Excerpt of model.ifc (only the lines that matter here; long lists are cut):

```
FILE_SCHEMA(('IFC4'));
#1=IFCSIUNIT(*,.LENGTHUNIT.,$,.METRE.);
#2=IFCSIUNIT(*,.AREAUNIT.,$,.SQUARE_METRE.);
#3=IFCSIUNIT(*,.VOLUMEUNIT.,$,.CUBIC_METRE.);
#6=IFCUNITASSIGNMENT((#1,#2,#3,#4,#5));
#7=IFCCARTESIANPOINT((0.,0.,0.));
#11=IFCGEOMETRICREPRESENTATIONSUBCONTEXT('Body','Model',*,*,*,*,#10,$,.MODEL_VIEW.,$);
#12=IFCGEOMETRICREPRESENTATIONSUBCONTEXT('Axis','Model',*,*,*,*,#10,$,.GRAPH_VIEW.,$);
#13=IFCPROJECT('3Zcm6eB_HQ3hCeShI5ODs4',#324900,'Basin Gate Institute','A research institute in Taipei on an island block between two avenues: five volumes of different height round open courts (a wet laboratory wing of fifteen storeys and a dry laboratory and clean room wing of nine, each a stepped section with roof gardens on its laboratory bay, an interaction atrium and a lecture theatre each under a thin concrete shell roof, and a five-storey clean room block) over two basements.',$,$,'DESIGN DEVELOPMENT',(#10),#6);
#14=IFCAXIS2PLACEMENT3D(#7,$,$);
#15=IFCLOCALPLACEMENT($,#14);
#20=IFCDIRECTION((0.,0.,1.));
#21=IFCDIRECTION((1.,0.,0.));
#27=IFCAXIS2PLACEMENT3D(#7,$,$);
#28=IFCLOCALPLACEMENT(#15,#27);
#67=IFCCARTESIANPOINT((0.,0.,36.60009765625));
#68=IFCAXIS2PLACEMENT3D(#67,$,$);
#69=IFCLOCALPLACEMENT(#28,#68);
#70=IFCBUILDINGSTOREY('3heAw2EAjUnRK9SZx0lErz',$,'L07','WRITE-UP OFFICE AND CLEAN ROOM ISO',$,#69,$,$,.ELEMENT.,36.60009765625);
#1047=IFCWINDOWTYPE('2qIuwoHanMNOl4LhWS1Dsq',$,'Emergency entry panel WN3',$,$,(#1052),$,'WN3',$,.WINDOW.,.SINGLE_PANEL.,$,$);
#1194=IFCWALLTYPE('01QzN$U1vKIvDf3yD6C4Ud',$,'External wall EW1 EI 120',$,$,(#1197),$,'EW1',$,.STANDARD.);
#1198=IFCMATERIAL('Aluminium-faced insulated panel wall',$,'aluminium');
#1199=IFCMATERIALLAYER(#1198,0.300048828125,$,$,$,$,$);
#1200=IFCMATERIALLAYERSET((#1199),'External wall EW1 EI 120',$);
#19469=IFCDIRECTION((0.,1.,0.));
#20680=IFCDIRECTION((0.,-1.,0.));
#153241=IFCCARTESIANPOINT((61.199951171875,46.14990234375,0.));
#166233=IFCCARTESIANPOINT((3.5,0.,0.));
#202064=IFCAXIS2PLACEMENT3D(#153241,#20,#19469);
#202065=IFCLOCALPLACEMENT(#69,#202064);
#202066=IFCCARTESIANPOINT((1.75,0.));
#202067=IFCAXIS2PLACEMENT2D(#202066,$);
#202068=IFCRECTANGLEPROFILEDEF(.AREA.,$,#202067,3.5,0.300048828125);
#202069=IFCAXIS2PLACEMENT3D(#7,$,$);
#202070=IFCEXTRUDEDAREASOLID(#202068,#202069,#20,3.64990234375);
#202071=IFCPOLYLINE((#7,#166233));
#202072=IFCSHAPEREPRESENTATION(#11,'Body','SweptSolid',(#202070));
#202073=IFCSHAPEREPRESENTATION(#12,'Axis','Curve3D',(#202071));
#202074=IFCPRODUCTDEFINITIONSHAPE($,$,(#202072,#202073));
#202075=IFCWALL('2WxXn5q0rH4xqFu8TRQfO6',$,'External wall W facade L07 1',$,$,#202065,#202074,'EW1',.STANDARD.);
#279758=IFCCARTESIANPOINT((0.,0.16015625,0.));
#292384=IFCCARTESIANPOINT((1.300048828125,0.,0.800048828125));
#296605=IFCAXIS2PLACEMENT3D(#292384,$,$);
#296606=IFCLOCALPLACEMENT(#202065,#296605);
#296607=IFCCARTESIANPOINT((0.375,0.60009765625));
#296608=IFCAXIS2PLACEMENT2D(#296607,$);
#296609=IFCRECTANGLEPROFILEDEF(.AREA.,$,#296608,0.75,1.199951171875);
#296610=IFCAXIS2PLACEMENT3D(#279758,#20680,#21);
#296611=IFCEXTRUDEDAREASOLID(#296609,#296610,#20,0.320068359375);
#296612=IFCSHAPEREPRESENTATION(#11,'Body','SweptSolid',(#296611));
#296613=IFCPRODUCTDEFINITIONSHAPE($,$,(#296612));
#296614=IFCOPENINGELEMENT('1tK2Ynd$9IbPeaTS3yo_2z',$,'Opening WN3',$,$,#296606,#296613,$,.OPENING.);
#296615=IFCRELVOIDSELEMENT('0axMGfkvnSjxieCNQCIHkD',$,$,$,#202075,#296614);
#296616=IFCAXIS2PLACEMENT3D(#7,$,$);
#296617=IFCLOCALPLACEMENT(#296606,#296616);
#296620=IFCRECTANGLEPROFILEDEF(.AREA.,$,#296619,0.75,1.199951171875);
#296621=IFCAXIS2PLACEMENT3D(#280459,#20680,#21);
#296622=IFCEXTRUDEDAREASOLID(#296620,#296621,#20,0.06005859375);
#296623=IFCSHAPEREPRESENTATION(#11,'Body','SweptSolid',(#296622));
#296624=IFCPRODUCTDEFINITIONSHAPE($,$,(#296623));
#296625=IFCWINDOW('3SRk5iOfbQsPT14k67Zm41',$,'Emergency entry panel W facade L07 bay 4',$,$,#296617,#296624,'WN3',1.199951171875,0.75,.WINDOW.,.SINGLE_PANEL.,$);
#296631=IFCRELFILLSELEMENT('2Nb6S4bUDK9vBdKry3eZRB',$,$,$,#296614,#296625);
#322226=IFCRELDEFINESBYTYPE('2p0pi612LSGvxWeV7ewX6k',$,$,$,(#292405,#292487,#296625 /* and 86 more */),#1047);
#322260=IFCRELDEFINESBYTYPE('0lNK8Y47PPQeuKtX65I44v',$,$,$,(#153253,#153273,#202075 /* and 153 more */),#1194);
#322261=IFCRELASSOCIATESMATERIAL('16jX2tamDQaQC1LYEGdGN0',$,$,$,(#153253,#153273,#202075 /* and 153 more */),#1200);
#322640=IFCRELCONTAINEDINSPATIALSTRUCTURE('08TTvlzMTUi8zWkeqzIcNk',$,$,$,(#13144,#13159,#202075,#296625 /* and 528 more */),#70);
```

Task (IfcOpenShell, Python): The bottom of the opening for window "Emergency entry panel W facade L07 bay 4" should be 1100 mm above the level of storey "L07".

```python
import numpy as np
import ifcopenshell
import ifcopenshell.api.geometry
import ifcopenshell.geom
import ifcopenshell.util.element
import ifcopenshell.util.placement
import ifcopenshell.util.shape
import ifcopenshell.util.unit

model = ifcopenshell.open("model.ifc")
unit_scale = ifcopenshell.util.unit.calculate_unit_scale(model)

window = model.by_guid("3SRk5iOfbQsPT14k67Zm41")
opening = window.FillsVoids[0].RelatingOpeningElement
storey = ifcopenshell.util.element.get_container(window, ifc_class="IfcBuildingStorey")
level = ifcopenshell.util.placement.get_local_placement(storey.ObjectPlacement)[2, 3]

# The opening's origin need not be at the sill, so measure its lowest point.
shape = ifcopenshell.geom.create_shape(ifcopenshell.geom.settings(), opening)
bottom = ifcopenshell.util.shape.get_shape_bottom_elevation(shape, shape.geometry) / unit_scale
dz = level + 1.1 / unit_scale - bottom

shift = np.array([0.0, 0.0, dz])
# The window is placed relative to its opening, so it follows when the opening moves.
matrix = ifcopenshell.util.placement.get_local_placement(opening.ObjectPlacement)
matrix[:3, 3] += shift
ifcopenshell.api.geometry.edit_object_placement(
    model, product=opening, matrix=matrix, is_si=False, should_transform_children=True
)

print(f"moved by {dz * unit_scale:+.3f} m")

model.write("model_v2.ifc")
```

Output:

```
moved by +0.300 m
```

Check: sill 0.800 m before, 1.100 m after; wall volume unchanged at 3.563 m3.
